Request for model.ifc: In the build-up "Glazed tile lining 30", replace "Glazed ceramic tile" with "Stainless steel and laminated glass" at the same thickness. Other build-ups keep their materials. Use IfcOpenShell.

First a look at what the model holds.

```python
import ifcopenshell
import ifcopenshell.util.element

model = ifcopenshell.open("model.ifc")
print(model.schema)
for layer_set in model.by_type("IfcMaterialLayerSet"):
    if layer_set.LayerSetName == "Glazed tile lining 30":
        for layer in layer_set.MaterialLayers:
            print(layer.id(), layer.Material and layer.Material.Name, layer.LayerThickness, sep=" | ")
        print(len(ifcopenshell.util.element.get_elements_by_material(model, layer_set)), "elements and types use it")
print(sorted(m.Name for m in model.by_type("IfcMaterial") if m.Name)[:60])
```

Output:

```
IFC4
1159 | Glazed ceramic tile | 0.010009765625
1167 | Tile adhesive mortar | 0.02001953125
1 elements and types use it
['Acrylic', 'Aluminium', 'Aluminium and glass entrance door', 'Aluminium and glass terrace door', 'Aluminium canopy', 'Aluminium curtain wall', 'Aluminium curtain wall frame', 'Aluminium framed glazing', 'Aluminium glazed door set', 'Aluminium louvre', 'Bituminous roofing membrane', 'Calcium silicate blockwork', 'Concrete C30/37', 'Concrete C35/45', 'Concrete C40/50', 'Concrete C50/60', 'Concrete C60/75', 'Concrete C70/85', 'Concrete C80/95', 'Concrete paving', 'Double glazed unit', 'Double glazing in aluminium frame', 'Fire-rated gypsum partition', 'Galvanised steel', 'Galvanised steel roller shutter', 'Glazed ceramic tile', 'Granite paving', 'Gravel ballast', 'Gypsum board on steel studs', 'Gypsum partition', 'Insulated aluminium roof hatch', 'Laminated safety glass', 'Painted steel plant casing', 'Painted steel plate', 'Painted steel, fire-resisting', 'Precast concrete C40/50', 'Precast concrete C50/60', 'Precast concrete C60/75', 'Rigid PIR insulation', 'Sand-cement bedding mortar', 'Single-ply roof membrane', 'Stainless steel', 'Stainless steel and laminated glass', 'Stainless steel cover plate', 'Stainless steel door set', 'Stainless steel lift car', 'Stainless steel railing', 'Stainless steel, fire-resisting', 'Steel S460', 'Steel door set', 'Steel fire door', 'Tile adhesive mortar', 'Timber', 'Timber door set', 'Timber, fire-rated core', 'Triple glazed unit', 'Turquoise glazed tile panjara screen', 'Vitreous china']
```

```python
import ifcopenshell
import ifcopenshell.api.material

model = ifcopenshell.open("model.ifc")

layer_set = next(s for s in model.by_type("IfcMaterialLayerSet") if s.LayerSetName == "Glazed tile lining 30")
layer = next(l for l in layer_set.MaterialLayers if l.Material and l.Material.Name == "Glazed ceramic tile")
material = next(m for m in model.by_type("IfcMaterial") if m.Name == "Stainless steel and laminated glass")

# Point this one layer at the other material; renaming the old one would change it everywhere.
ifcopenshell.api.material.edit_layer(model, layer=layer, attributes={}, material=material)

print([l.Material.Name if l.Material else None for l in layer_set.MaterialLayers])

model.write("model_rev.ifc")
```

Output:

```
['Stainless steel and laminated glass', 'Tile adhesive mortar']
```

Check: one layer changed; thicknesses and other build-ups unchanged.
